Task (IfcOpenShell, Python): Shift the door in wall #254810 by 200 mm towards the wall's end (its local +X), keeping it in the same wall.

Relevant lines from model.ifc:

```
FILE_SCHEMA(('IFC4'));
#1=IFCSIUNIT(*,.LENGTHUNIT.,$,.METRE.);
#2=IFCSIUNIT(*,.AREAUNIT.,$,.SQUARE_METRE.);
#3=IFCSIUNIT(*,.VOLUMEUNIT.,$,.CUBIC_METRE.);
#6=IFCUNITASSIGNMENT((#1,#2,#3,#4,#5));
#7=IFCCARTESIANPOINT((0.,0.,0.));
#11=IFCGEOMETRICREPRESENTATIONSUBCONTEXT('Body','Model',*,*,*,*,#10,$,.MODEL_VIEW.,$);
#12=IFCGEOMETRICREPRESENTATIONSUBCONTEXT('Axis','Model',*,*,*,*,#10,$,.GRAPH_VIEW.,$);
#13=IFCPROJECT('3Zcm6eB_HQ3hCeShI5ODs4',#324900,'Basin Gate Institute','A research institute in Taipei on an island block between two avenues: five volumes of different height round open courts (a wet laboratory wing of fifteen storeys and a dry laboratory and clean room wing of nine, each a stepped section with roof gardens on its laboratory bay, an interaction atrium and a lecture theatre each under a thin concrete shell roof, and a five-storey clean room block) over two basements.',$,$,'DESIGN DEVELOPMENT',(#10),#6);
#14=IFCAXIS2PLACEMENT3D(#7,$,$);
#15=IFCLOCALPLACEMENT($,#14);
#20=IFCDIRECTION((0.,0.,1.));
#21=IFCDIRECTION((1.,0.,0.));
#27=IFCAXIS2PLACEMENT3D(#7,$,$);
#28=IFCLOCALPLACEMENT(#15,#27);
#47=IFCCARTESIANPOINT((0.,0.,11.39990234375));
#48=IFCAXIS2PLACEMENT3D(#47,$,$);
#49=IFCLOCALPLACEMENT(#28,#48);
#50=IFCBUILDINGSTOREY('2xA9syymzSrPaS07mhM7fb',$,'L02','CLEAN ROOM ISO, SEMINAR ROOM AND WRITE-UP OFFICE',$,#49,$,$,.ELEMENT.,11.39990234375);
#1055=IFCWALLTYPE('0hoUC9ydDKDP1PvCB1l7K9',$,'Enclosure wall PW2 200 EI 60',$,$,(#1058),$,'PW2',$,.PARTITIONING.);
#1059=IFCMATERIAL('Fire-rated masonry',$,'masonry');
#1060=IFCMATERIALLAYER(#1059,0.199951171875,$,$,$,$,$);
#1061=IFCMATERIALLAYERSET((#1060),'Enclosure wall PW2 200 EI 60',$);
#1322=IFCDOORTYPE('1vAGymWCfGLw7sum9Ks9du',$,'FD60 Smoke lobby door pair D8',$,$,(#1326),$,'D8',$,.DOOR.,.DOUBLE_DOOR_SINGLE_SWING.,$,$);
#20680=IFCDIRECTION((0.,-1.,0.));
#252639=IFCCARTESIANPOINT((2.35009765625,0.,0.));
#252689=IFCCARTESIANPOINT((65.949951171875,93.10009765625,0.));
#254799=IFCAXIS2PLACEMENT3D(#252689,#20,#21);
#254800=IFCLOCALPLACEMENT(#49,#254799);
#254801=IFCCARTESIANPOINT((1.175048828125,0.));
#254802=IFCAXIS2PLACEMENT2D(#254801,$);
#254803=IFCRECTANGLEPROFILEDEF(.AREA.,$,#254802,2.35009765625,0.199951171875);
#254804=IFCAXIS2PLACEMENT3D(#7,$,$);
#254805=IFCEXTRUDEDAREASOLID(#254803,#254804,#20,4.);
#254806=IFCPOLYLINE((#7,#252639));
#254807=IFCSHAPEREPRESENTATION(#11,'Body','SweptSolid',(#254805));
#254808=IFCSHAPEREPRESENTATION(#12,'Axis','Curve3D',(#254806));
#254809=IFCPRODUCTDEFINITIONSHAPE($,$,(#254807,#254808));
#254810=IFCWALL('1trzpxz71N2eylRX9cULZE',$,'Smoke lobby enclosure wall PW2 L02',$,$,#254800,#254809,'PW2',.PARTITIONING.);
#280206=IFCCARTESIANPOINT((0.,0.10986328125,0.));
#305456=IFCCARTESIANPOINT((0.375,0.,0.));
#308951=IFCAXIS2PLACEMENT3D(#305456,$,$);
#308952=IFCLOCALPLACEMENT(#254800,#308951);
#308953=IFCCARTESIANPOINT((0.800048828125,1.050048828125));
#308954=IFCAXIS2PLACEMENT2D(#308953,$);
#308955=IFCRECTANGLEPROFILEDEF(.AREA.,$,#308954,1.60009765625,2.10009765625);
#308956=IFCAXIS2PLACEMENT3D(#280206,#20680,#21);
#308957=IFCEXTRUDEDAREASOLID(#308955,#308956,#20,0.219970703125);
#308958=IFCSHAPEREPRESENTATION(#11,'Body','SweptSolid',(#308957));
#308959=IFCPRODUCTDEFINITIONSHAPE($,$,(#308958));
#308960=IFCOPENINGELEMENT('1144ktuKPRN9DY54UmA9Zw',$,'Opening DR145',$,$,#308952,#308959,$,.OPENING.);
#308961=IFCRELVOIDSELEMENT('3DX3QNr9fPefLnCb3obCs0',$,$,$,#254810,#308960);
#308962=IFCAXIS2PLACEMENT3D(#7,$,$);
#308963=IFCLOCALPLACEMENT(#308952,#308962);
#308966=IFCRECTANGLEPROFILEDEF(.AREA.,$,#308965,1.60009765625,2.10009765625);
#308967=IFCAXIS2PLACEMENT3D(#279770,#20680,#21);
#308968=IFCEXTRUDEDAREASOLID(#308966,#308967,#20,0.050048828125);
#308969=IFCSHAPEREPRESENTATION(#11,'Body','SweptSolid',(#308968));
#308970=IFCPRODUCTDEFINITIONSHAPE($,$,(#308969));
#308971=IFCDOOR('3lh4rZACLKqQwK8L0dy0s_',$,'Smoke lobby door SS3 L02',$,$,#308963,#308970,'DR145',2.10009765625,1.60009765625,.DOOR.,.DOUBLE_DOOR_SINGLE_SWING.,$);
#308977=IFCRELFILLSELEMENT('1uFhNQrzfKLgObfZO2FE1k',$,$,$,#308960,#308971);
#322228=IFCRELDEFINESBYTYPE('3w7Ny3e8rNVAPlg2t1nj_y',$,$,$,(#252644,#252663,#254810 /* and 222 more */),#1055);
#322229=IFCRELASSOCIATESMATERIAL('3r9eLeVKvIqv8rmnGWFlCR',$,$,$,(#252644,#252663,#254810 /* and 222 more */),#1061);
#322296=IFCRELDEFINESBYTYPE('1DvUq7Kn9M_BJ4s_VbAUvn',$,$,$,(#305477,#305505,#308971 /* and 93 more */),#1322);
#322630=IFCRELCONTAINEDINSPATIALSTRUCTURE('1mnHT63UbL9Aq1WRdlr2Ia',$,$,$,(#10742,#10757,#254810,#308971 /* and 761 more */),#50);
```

```python
import ifcopenshell
import ifcopenshell.api.geometry
import ifcopenshell.util.placement
import ifcopenshell.util.unit

model = ifcopenshell.open("model.ifc")
unit_scale = ifcopenshell.util.unit.calculate_unit_scale(model)

door = model.by_guid("3lh4rZACLKqQwK8L0dy0s_")
opening = door.FillsVoids[0].RelatingOpeningElement
wall = opening.VoidsElements[0].RelatingBuildingElement

wall_matrix = ifcopenshell.util.placement.get_local_placement(wall.ObjectPlacement)
shift = wall_matrix[:3, 0] * 0.2 / unit_scale
before = ifcopenshell.util.placement.get_local_placement(door.ObjectPlacement)[:3, 3].copy()

# The door is placed relative to its opening, so it follows when the opening moves.
matrix = ifcopenshell.util.placement.get_local_placement(opening.ObjectPlacement)
matrix[:3, 3] += shift
ifcopenshell.api.geometry.edit_object_placement(
    model, product=opening, matrix=matrix, is_si=False, should_transform_children=True
)

after = ifcopenshell.util.placement.get_local_placement(door.ObjectPlacement)[:3, 3]
print("door moved by", (after - before).round(3) + 0.0)

model.write("model-out.ifc")
```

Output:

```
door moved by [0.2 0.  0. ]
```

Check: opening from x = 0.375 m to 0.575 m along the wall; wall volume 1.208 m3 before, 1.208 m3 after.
